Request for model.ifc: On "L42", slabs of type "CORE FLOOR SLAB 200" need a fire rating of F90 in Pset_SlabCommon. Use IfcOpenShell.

First a look at what the model holds.

```python
import ifcopenshell
import ifcopenshell.util.element

model = ifcopenshell.open("model.ifc")
print(model.schema)
storey = next(s for s in model.by_type("IfcBuildingStorey") if s.Name == "L42")
slabs = [e for e in ifcopenshell.util.element.get_decomposition(storey) if e.is_a("IfcSlab")]
seen = {}
for e in slabs:
    element_type = ifcopenshell.util.element.get_type(e)
    key = (element_type.Name if element_type != e and element_type else None, ifcopenshell.util.element.get_pset(e, "Pset_SlabCommon", "FireRating"))
    seen[key] = seen.get(key, 0) + 1
for (name, value), count in sorted(seen.items(), key=str):
    print(count, "x", name, "|", value)
```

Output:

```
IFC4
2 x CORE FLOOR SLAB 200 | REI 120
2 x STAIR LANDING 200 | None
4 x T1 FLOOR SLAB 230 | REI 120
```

```python
import ifcopenshell
import ifcopenshell.api.pset
import ifcopenshell.util.element

model = ifcopenshell.open("model.ifc")

storey = next(s for s in model.by_type("IfcBuildingStorey") if s.Name == "L42")
slabs = [e for e in ifcopenshell.util.element.get_decomposition(storey) if e.is_a("IfcSlab")]

count = 0
for e in slabs:
    element_type = ifcopenshell.util.element.get_type(e)
    if element_type in (None, e) or element_type.Name != "CORE FLOOR SLAB 200":
        continue
    found = ifcopenshell.util.element.get_pset(e, "Pset_SlabCommon", should_inherit=False)
    if found:
        pset = model.by_id(found["id"])
        if len(ifcopenshell.util.element.get_elements_by_pset(pset)) > 1:
            pset = ifcopenshell.api.pset.unshare_pset(model, products=[e], pset=pset)[0]
    else:
        pset = ifcopenshell.api.pset.add_pset(model, product=e, name="Pset_SlabCommon")
    ifcopenshell.api.pset.edit_pset(model, pset=pset, properties={"FireRating": "F90"})
    count += 1

print(count, "slabs updated")

model.write("model_rev.ifc")
```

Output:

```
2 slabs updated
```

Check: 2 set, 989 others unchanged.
